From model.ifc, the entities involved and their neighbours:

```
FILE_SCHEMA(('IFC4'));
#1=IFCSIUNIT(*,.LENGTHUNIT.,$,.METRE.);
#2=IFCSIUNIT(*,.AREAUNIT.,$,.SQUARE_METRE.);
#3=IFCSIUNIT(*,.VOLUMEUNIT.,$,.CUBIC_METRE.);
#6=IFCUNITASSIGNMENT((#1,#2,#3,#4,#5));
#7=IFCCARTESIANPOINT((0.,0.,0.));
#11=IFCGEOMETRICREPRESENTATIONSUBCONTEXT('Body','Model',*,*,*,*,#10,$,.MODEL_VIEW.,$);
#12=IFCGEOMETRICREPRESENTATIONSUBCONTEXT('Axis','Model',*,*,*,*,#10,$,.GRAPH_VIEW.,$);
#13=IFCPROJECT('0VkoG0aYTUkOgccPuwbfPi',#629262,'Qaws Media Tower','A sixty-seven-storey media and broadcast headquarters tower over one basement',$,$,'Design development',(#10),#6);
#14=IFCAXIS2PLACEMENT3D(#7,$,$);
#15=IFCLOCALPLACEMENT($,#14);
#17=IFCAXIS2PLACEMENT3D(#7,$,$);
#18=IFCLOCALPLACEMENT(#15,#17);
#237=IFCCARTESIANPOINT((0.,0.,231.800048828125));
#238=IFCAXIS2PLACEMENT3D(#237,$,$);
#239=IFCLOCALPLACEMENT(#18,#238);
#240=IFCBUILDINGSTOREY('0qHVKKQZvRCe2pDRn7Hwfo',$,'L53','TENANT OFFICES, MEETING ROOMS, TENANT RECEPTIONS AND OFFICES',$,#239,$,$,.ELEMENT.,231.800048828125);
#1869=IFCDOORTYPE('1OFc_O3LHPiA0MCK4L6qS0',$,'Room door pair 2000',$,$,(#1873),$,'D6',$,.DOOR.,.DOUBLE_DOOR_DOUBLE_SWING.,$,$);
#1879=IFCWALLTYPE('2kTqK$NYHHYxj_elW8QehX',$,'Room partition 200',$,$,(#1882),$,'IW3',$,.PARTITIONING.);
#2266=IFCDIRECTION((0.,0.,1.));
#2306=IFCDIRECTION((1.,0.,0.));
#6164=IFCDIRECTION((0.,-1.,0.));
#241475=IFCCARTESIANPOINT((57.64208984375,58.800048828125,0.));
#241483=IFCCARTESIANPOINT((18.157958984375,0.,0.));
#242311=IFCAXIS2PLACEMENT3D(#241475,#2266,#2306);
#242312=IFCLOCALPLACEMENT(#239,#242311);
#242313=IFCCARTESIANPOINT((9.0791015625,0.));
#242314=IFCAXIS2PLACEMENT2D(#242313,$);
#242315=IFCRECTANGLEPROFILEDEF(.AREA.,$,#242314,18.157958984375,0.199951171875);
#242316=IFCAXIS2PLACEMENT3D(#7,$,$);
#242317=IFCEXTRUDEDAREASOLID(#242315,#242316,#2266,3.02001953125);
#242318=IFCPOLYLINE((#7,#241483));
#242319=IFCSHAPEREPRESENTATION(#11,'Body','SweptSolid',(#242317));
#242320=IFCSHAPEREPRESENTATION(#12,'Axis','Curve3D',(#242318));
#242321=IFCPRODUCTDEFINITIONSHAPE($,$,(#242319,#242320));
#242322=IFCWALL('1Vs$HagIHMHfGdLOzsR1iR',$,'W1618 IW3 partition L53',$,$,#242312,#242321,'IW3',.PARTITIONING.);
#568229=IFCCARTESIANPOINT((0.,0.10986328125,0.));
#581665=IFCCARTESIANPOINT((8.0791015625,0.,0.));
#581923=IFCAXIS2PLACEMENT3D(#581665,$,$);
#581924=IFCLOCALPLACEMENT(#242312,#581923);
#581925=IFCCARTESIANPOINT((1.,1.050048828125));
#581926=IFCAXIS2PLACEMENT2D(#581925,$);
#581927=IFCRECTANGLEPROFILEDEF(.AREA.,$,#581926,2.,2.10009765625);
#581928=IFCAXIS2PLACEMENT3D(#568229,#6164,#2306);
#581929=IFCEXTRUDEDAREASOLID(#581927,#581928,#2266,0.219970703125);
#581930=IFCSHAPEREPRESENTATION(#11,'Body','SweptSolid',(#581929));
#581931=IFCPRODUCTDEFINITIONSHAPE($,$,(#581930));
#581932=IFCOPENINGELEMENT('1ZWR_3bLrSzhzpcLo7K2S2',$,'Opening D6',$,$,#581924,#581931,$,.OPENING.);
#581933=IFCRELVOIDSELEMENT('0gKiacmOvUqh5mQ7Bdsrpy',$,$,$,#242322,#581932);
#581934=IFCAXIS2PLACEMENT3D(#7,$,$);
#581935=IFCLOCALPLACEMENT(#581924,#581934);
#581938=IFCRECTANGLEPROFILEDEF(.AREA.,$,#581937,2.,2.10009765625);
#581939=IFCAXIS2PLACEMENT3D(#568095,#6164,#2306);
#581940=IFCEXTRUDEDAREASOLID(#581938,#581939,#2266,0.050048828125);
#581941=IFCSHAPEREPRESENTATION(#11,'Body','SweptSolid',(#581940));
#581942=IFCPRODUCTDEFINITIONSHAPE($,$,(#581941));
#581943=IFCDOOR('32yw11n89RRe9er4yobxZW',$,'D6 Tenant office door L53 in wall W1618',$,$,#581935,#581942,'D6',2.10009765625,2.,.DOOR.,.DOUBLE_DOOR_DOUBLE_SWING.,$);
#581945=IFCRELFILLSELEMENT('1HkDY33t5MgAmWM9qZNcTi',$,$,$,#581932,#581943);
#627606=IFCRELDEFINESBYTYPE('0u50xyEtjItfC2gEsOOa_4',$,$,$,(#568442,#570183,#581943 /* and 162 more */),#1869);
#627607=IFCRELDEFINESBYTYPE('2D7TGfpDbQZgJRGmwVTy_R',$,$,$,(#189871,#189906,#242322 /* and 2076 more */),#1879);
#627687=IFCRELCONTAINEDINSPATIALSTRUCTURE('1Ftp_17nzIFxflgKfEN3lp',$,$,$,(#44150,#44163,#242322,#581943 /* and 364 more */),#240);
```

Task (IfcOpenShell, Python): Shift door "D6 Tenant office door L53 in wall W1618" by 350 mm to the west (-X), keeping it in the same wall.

```python
import ifcopenshell
import ifcopenshell.api.geometry
import ifcopenshell.util.placement

model = ifcopenshell.open("model.ifc")

door = model.by_id(581943)
opening = door.FillsVoids[0].RelatingOpeningElement
wall = opening.VoidsElements[0].RelatingBuildingElement

wall_matrix = ifcopenshell.util.placement.get_local_placement(wall.ObjectPlacement)
shift = wall_matrix[:3, 0] * -0.35
before = ifcopenshell.util.placement.get_local_placement(door.ObjectPlacement)[:3, 3].copy()

# The door is placed relative to its opening, so it follows when the opening moves.
matrix = ifcopenshell.util.placement.get_local_placement(opening.ObjectPlacement)
matrix[:3, 3] += shift
ifcopenshell.api.geometry.edit_object_placement(
    model, product=opening, matrix=matrix, is_si=False, should_transform_children=True
)

after = ifcopenshell.util.placement.get_local_placement(door.ObjectPlacement)[:3, 3]
print("door moved by", (after - before).round(3) + 0.0)

model.write("model-out.ifc")
```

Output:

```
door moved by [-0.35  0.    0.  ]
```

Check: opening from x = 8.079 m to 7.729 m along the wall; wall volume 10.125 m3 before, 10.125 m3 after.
